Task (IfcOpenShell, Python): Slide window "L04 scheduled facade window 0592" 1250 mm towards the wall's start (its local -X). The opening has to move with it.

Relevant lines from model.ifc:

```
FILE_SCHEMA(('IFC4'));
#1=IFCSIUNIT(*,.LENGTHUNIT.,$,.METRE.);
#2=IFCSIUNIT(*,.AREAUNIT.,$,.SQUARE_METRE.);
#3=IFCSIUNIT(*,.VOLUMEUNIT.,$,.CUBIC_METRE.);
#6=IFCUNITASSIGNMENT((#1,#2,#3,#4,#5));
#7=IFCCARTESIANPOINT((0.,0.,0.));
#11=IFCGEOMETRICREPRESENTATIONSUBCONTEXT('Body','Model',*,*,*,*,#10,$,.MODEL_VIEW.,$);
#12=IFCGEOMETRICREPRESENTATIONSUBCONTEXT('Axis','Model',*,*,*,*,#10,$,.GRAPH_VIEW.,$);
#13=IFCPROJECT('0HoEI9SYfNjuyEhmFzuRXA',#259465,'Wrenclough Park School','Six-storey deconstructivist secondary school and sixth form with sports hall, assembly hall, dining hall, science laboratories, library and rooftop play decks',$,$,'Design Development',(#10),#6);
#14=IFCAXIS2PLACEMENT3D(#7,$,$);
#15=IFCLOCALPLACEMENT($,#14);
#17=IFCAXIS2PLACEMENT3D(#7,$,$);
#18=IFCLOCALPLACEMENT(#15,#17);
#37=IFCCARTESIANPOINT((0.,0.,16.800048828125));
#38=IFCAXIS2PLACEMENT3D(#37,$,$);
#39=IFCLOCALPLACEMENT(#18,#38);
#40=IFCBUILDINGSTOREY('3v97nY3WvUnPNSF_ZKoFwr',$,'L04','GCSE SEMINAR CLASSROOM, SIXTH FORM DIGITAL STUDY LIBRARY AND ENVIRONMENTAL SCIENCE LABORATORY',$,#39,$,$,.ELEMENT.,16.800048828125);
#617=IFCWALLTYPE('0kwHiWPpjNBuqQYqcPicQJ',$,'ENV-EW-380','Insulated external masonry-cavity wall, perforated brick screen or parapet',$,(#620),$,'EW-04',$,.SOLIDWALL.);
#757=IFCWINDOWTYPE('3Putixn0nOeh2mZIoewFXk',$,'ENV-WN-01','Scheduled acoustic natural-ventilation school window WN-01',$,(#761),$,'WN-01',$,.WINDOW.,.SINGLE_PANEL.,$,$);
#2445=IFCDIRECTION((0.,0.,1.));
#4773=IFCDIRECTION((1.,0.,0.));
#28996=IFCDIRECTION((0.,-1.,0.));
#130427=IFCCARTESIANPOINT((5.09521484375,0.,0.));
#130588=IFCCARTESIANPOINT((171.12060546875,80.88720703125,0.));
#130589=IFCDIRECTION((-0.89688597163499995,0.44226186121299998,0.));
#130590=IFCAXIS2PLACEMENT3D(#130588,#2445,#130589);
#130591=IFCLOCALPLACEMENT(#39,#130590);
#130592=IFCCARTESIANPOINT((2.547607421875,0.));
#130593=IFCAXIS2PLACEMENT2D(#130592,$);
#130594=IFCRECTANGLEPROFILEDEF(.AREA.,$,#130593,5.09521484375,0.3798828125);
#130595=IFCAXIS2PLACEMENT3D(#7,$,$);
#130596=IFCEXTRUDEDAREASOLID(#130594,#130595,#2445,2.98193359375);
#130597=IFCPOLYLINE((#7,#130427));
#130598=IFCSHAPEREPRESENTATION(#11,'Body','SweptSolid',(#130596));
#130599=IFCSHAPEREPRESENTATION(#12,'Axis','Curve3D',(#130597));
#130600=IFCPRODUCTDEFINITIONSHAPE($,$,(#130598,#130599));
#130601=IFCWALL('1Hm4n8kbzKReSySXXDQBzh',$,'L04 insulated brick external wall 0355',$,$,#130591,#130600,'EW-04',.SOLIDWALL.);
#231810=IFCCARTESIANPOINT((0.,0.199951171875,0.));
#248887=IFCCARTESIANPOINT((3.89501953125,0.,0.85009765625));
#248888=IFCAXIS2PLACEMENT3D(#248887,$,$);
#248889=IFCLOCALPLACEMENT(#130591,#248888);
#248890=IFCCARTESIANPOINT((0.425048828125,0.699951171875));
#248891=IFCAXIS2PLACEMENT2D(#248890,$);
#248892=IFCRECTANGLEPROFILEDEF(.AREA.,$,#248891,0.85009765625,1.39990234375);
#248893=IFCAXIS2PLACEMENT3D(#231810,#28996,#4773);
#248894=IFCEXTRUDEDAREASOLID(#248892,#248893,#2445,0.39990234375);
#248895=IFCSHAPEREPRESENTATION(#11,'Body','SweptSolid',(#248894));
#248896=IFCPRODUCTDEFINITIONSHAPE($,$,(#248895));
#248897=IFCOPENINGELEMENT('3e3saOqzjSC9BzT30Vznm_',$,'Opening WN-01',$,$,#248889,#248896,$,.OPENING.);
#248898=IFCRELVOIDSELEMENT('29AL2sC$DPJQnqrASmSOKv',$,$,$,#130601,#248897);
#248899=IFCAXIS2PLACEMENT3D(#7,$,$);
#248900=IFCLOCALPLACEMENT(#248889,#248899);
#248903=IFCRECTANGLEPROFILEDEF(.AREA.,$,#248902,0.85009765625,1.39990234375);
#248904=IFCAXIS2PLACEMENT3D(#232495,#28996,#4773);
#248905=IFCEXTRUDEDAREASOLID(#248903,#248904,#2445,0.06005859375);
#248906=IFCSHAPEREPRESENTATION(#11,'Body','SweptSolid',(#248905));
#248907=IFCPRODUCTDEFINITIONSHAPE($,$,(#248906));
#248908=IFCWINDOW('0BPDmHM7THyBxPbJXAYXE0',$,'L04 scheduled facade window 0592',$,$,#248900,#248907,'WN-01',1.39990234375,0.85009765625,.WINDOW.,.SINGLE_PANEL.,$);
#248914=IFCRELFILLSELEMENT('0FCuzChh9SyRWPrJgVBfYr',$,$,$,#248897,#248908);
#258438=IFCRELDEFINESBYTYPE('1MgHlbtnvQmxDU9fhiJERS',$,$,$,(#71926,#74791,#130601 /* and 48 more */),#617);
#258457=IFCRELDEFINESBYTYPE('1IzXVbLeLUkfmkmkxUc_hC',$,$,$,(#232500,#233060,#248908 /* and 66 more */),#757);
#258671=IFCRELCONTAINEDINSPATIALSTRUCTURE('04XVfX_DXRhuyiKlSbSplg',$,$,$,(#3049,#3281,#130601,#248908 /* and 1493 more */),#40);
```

```python
import ifcopenshell
import ifcopenshell.api.geometry
import ifcopenshell.util.placement

model = ifcopenshell.open("model.ifc")

window = model.by_guid("0BPDmHM7THyBxPbJXAYXE0")
opening = window.FillsVoids[0].RelatingOpeningElement
wall = opening.VoidsElements[0].RelatingBuildingElement

wall_matrix = ifcopenshell.util.placement.get_local_placement(wall.ObjectPlacement)
shift = wall_matrix[:3, 0] * -1.25
before = ifcopenshell.util.placement.get_local_placement(window.ObjectPlacement)[:3, 3].copy()

# The window is placed relative to its opening, so it follows when the opening moves.
matrix = ifcopenshell.util.placement.get_local_placement(opening.ObjectPlacement)
matrix[:3, 3] += shift
ifcopenshell.api.geometry.edit_object_placement(
    model, product=opening, matrix=matrix, is_si=False, should_transform_children=True
)

after = ifcopenshell.util.placement.get_local_placement(window.ObjectPlacement)[:3, 3]
print("window moved by", (after - before).round(3) + 0.0)

model.write("model-out.ifc")
```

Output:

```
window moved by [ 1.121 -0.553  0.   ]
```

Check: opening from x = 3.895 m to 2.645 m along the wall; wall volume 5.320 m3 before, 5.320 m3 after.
